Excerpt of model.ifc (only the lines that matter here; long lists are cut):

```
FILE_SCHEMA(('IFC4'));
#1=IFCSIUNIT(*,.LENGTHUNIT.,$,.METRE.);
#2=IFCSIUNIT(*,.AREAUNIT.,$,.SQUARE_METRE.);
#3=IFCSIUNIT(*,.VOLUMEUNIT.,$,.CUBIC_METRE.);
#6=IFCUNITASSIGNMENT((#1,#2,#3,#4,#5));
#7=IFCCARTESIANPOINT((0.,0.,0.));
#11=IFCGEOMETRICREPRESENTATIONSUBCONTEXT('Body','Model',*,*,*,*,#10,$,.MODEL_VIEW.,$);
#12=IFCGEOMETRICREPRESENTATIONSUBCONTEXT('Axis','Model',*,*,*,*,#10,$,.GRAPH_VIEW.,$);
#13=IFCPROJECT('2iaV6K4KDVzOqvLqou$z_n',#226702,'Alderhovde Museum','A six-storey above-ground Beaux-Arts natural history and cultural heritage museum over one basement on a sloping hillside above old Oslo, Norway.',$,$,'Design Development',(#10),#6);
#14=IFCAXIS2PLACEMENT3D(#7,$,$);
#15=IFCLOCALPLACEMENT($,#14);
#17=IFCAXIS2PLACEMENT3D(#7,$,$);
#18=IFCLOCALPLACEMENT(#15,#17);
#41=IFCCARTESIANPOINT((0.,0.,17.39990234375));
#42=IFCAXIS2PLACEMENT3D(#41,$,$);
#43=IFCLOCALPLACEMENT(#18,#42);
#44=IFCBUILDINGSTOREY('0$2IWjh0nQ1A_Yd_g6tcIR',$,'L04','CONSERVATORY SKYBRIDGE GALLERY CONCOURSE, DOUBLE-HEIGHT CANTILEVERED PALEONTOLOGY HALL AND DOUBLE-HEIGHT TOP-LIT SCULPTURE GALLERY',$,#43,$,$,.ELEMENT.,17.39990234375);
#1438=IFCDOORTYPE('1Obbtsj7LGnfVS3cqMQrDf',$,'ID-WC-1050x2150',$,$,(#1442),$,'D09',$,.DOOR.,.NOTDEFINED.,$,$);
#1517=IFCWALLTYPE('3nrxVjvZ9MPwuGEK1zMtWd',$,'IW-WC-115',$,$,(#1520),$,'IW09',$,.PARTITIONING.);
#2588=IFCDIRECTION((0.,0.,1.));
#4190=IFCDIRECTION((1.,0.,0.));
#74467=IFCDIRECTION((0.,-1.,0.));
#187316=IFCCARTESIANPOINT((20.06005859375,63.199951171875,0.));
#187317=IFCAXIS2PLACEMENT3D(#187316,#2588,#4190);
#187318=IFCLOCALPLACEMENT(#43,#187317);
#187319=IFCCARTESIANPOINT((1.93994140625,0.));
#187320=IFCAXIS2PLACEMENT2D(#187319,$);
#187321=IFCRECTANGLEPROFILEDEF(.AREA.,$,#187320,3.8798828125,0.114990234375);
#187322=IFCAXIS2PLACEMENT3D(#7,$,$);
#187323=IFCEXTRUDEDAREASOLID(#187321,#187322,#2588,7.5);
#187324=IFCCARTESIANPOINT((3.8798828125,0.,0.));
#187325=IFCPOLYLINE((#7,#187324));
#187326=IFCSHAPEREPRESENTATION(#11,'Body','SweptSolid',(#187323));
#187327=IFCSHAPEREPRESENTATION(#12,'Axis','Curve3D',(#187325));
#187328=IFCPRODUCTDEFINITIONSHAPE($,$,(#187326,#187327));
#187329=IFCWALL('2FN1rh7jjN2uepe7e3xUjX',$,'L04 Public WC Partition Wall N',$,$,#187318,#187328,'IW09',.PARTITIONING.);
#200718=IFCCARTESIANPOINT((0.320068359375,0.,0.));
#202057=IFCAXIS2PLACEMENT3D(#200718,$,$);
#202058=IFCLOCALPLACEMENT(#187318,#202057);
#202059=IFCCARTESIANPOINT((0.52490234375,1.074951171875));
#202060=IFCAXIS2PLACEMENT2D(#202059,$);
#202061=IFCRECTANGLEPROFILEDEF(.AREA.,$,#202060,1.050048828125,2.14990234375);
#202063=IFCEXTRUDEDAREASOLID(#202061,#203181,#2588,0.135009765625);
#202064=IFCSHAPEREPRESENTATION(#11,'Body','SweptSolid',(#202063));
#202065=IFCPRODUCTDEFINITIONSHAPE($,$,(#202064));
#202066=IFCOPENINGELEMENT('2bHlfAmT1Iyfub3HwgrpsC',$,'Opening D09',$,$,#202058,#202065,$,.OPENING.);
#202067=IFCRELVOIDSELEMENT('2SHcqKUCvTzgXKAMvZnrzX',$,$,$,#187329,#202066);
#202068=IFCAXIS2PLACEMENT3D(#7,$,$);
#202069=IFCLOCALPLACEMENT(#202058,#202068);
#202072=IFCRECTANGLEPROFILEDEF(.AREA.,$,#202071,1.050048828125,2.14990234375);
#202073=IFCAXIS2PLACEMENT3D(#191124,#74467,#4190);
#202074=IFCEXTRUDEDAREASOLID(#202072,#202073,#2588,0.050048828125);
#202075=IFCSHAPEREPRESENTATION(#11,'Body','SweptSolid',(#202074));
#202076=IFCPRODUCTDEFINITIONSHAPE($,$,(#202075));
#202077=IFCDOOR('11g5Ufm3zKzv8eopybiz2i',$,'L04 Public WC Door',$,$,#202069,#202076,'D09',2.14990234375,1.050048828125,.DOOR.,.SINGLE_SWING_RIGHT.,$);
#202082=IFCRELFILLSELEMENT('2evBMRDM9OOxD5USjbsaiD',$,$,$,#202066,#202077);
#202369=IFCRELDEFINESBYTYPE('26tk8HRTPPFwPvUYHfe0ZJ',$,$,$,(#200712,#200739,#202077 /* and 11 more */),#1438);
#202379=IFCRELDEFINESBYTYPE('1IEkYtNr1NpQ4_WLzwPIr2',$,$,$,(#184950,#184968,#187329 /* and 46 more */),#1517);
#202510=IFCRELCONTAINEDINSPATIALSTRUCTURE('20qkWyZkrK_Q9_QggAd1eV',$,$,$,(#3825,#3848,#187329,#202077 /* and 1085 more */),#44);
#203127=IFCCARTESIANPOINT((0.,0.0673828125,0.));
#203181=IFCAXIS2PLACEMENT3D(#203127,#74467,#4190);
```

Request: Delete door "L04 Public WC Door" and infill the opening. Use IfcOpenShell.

```python
import ifcopenshell
import ifcopenshell.api.feature
import ifcopenshell.api.root
import ifcopenshell.geom
import ifcopenshell.util.shape

model = ifcopenshell.open("model.ifc")
settings = ifcopenshell.geom.settings()


def volume(element):
    """Net volume in cubic metres, openings subtracted."""
    shape = ifcopenshell.geom.create_shape(settings, element)
    return ifcopenshell.util.shape.get_volume(shape.geometry)


door = model.by_guid("11g5Ufm3zKzv8eopybiz2i")
opening = door.FillsVoids[0].RelatingOpeningElement
wall = opening.VoidsElements[0].RelatingBuildingElement
before = volume(wall)

ifcopenshell.api.root.remove_product(model, product=door)
ifcopenshell.api.feature.remove_feature(model, feature=opening)

after = volume(wall)

print(f"wall volume {before:.3f} -> {after:.3f} m3")

model.write("model_rev.ifc")
```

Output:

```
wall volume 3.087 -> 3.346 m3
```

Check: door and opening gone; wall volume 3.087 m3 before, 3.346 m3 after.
